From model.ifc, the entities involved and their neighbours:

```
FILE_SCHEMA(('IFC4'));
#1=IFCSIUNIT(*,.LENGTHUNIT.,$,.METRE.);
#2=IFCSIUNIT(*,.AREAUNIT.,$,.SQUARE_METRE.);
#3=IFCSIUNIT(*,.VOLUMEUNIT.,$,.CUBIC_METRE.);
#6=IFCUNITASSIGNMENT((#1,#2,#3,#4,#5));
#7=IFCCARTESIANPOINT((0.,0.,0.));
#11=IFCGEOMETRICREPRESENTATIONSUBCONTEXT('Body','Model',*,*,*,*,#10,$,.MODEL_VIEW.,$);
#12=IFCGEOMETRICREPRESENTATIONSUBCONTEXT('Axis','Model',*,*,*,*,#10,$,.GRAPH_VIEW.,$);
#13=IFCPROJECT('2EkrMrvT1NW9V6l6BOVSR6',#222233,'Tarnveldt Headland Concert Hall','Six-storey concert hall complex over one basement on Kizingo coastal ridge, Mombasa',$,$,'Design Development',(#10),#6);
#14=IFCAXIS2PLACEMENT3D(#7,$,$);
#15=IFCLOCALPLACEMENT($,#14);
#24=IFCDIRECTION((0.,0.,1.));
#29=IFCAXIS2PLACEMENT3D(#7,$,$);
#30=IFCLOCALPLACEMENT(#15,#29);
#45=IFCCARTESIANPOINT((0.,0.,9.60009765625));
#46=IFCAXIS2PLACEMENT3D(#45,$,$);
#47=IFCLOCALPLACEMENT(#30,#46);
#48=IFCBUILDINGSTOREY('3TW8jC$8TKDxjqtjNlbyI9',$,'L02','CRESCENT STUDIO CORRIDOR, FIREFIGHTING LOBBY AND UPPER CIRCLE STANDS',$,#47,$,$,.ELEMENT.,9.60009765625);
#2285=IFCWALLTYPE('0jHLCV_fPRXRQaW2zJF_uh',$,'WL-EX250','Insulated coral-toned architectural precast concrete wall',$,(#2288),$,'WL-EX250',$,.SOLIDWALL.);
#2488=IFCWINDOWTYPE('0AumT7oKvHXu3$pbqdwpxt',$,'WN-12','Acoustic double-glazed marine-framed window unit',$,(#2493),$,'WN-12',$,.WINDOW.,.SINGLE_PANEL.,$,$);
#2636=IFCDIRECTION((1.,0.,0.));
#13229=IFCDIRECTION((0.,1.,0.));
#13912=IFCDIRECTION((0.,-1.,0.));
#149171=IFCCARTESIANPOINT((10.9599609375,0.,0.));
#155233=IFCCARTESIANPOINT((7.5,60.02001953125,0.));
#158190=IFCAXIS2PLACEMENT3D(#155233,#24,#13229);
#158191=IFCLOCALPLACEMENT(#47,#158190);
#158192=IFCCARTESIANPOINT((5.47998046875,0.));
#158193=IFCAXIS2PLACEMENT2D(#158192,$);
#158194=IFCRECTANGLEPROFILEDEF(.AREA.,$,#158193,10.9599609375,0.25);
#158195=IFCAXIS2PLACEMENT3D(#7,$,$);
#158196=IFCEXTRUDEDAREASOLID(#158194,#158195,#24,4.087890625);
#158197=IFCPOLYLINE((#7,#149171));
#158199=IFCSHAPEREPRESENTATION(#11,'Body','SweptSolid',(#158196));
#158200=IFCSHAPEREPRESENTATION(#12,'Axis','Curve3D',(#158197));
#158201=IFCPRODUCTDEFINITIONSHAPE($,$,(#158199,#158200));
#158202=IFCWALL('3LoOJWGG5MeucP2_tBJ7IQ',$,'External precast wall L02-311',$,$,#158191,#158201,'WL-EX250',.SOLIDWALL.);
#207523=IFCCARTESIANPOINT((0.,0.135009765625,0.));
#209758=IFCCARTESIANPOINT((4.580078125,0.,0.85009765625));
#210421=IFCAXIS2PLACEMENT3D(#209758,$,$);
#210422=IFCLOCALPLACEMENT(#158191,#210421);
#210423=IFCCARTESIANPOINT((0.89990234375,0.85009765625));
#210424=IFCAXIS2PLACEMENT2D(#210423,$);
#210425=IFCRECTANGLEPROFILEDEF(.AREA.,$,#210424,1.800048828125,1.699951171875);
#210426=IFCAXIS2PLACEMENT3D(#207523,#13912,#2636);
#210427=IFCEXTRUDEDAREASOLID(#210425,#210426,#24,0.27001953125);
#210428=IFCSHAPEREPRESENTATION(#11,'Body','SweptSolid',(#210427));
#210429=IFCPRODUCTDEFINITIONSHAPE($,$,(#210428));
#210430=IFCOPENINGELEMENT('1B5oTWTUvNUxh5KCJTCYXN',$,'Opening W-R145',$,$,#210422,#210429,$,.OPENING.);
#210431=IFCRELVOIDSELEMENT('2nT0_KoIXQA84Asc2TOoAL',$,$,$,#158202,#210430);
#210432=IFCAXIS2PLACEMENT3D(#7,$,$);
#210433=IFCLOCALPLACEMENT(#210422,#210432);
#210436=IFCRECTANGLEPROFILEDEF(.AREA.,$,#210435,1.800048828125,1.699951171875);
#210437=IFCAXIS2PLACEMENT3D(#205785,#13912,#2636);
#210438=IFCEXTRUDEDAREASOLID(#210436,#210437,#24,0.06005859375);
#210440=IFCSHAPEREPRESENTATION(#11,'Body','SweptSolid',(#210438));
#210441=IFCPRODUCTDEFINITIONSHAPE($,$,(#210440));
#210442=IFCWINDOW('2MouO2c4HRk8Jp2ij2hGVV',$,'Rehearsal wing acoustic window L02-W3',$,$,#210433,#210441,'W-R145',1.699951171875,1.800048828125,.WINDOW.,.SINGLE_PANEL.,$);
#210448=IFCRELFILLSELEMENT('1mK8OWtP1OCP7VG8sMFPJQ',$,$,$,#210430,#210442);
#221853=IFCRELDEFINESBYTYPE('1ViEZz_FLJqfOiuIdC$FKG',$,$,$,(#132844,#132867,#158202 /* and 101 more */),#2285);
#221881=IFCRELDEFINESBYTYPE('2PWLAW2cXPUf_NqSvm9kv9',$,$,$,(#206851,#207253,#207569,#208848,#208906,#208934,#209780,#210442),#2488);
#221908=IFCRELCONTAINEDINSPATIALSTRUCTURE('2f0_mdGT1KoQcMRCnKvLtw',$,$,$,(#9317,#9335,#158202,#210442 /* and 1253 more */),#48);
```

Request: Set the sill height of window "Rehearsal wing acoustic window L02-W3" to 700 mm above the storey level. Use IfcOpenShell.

```python
import numpy as np
import ifcopenshell
import ifcopenshell.api.geometry
import ifcopenshell.geom
import ifcopenshell.util.element
import ifcopenshell.util.placement
import ifcopenshell.util.shape
import ifcopenshell.util.unit

model = ifcopenshell.open("model.ifc")
unit_scale = ifcopenshell.util.unit.calculate_unit_scale(model)

window = model.by_id(210442)
opening = window.FillsVoids[0].RelatingOpeningElement
storey = ifcopenshell.util.element.get_container(window, ifc_class="IfcBuildingStorey")
level = ifcopenshell.util.placement.get_local_placement(storey.ObjectPlacement)[2, 3]

# The opening's origin need not be at the sill, so measure its lowest point.
shape = ifcopenshell.geom.create_shape(ifcopenshell.geom.settings(), opening)
bottom = ifcopenshell.util.shape.get_shape_bottom_elevation(shape, shape.geometry) / unit_scale
dz = level + 0.7 / unit_scale - bottom

shift = np.array([0.0, 0.0, dz])
# The window is placed relative to its opening, so it follows when the opening moves.
matrix = ifcopenshell.util.placement.get_local_placement(opening.ObjectPlacement)
matrix[:3, 3] += shift
ifcopenshell.api.geometry.edit_object_placement(
    model, product=opening, matrix=matrix, is_si=False, should_transform_children=True
)

print(f"moved by {dz * unit_scale:+.3f} m")

model.write("model-out.ifc")
```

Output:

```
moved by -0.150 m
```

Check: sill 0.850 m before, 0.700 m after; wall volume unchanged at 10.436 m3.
